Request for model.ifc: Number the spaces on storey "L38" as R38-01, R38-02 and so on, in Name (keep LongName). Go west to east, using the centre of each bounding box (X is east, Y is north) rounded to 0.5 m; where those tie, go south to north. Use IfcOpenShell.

First a look at what the model holds.

```python
import ifcopenshell
import ifcopenshell.util.element
import ifcopenshell.util.placement

model = ifcopenshell.open("model.ifc")
print(model.schema)
storey = next(s for s in model.by_type("IfcBuildingStorey") if s.Name == "L38")
spaces = [e for e in ifcopenshell.util.element.get_decomposition(storey) if e.is_a("IfcSpace")]
for e in sorted(spaces, key=lambda e: e.id()):
    origin = ifcopenshell.util.placement.get_local_placement(e.ObjectPlacement)[:3, 3]
    print(e.id(), e.Name, e.LongName, origin.round(2) + 0.0, sep=" | ")
```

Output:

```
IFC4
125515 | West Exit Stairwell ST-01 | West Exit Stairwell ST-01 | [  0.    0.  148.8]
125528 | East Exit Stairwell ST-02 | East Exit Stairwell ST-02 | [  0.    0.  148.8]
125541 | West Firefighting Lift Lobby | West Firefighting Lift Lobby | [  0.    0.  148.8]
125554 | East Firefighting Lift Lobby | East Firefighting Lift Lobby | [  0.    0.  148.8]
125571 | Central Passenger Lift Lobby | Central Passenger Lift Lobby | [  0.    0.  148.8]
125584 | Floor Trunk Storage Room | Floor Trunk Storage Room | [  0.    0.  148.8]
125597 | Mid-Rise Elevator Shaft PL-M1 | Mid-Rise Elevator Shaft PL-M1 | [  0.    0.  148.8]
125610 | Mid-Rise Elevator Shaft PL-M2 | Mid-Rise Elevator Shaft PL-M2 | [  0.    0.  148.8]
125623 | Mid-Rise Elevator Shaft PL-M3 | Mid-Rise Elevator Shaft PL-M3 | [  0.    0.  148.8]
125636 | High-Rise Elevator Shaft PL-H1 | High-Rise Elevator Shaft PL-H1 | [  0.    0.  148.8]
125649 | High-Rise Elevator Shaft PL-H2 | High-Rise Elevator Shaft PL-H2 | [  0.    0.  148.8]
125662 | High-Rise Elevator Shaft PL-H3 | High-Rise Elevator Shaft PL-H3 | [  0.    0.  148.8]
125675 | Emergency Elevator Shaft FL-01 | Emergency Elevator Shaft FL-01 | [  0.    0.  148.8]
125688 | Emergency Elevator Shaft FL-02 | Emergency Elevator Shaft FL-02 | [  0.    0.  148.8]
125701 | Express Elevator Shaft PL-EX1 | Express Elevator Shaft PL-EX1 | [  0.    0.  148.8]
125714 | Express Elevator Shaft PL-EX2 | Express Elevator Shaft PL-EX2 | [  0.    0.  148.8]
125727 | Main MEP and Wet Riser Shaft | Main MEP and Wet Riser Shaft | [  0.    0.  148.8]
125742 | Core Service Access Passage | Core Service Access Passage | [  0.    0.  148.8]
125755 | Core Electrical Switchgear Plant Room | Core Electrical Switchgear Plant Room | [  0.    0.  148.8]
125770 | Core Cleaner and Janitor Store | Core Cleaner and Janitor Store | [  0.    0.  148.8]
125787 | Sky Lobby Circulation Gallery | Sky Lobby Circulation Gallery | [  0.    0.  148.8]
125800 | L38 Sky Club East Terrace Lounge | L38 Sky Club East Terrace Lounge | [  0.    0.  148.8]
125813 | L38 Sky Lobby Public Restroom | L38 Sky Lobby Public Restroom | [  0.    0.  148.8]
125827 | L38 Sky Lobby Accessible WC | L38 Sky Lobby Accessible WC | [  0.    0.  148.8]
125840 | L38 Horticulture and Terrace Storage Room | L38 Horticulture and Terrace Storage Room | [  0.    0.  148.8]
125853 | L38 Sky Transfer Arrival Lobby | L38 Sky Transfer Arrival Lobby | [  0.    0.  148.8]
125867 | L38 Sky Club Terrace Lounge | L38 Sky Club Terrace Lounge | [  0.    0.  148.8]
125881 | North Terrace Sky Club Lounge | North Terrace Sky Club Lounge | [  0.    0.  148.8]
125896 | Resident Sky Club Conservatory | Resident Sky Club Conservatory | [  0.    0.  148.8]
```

```python
import ifcopenshell
import ifcopenshell.geom
import ifcopenshell.util.element
import ifcopenshell.util.shape

model = ifcopenshell.open("model.ifc")
settings = ifcopenshell.geom.settings()
settings.set("use-world-coords", True)


def centre(element):
    shape = ifcopenshell.geom.create_shape(settings, element)
    return ifcopenshell.util.shape.get_bbox_centroid(shape.geometry)


storey = next(s for s in model.by_type("IfcBuildingStorey") if s.Name == "L38")
spaces = [e for e in ifcopenshell.util.element.get_decomposition(storey) if e.is_a("IfcSpace")]

# Insertion points can sit at a corner or the storey origin, so sort by the geometry (in metres).
centres = {e: centre(e) for e in spaces}
spaces.sort(key=lambda e: (round(centres[e][0] / 0.5), centres[e][1]))

for i, e in enumerate(spaces, start=1):
    number = f"R38-{i:02d}"
    e.Name = number
    print(e.id(), number)

model.write("model_rev.ifc")
```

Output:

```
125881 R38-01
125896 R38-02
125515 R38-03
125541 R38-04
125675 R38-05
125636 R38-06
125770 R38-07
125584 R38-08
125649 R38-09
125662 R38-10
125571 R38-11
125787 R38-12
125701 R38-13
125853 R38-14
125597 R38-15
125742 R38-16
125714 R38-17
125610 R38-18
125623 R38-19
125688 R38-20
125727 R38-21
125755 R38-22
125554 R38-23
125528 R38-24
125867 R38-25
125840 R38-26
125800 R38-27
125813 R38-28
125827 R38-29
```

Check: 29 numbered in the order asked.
